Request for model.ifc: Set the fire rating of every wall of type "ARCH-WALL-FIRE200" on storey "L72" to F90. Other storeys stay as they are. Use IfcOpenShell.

First a look at what the model holds.

```python
import ifcopenshell
import ifcopenshell.util.element

model = ifcopenshell.open("model.ifc")
print(model.schema)
storey = next(s for s in model.by_type("IfcBuildingStorey") if s.Name == "L72")
walls = [e for e in ifcopenshell.util.element.get_decomposition(storey) if e.is_a("IfcWall")]
seen = {}
for e in walls:
    element_type = ifcopenshell.util.element.get_type(e)
    key = (element_type.Name if element_type != e and element_type else None, ifcopenshell.util.element.get_pset(e, "Pset_WallCommon", "FireRating"))
    seen[key] = seen.get(key, 0) + 1
for (name, value), count in sorted(seen.items(), key=str):
    print(count, "x", name, "|", value)
```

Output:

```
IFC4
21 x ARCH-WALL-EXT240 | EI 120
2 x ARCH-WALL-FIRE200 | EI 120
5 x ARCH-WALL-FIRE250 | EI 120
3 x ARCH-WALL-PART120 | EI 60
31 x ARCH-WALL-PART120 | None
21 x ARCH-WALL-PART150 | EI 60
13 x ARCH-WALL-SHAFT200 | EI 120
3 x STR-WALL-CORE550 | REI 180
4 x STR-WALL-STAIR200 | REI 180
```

```python
import ifcopenshell
import ifcopenshell.api.pset
import ifcopenshell.util.element

model = ifcopenshell.open("model.ifc")

storey = next(s for s in model.by_type("IfcBuildingStorey") if s.Name == "L72")
walls = [e for e in ifcopenshell.util.element.get_decomposition(storey) if e.is_a("IfcWall")]

count = 0
for e in walls:
    element_type = ifcopenshell.util.element.get_type(e)
    if element_type in (None, e) or element_type.Name != "ARCH-WALL-FIRE200":
        continue
    found = ifcopenshell.util.element.get_pset(e, "Pset_WallCommon", should_inherit=False)
    if found:
        pset = model.by_id(found["id"])
        if len(ifcopenshell.util.element.get_elements_by_pset(pset)) > 1:
            pset = ifcopenshell.api.pset.unshare_pset(model, products=[e], pset=pset)[0]
    else:
        pset = ifcopenshell.api.pset.add_pset(model, product=e, name="Pset_WallCommon")
    ifcopenshell.api.pset.edit_pset(model, pset=pset, properties={"FireRating": "F90"})
    count += 1

print(count, "walls updated")

model.write("model_v2.ifc")
```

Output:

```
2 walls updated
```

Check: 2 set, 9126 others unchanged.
